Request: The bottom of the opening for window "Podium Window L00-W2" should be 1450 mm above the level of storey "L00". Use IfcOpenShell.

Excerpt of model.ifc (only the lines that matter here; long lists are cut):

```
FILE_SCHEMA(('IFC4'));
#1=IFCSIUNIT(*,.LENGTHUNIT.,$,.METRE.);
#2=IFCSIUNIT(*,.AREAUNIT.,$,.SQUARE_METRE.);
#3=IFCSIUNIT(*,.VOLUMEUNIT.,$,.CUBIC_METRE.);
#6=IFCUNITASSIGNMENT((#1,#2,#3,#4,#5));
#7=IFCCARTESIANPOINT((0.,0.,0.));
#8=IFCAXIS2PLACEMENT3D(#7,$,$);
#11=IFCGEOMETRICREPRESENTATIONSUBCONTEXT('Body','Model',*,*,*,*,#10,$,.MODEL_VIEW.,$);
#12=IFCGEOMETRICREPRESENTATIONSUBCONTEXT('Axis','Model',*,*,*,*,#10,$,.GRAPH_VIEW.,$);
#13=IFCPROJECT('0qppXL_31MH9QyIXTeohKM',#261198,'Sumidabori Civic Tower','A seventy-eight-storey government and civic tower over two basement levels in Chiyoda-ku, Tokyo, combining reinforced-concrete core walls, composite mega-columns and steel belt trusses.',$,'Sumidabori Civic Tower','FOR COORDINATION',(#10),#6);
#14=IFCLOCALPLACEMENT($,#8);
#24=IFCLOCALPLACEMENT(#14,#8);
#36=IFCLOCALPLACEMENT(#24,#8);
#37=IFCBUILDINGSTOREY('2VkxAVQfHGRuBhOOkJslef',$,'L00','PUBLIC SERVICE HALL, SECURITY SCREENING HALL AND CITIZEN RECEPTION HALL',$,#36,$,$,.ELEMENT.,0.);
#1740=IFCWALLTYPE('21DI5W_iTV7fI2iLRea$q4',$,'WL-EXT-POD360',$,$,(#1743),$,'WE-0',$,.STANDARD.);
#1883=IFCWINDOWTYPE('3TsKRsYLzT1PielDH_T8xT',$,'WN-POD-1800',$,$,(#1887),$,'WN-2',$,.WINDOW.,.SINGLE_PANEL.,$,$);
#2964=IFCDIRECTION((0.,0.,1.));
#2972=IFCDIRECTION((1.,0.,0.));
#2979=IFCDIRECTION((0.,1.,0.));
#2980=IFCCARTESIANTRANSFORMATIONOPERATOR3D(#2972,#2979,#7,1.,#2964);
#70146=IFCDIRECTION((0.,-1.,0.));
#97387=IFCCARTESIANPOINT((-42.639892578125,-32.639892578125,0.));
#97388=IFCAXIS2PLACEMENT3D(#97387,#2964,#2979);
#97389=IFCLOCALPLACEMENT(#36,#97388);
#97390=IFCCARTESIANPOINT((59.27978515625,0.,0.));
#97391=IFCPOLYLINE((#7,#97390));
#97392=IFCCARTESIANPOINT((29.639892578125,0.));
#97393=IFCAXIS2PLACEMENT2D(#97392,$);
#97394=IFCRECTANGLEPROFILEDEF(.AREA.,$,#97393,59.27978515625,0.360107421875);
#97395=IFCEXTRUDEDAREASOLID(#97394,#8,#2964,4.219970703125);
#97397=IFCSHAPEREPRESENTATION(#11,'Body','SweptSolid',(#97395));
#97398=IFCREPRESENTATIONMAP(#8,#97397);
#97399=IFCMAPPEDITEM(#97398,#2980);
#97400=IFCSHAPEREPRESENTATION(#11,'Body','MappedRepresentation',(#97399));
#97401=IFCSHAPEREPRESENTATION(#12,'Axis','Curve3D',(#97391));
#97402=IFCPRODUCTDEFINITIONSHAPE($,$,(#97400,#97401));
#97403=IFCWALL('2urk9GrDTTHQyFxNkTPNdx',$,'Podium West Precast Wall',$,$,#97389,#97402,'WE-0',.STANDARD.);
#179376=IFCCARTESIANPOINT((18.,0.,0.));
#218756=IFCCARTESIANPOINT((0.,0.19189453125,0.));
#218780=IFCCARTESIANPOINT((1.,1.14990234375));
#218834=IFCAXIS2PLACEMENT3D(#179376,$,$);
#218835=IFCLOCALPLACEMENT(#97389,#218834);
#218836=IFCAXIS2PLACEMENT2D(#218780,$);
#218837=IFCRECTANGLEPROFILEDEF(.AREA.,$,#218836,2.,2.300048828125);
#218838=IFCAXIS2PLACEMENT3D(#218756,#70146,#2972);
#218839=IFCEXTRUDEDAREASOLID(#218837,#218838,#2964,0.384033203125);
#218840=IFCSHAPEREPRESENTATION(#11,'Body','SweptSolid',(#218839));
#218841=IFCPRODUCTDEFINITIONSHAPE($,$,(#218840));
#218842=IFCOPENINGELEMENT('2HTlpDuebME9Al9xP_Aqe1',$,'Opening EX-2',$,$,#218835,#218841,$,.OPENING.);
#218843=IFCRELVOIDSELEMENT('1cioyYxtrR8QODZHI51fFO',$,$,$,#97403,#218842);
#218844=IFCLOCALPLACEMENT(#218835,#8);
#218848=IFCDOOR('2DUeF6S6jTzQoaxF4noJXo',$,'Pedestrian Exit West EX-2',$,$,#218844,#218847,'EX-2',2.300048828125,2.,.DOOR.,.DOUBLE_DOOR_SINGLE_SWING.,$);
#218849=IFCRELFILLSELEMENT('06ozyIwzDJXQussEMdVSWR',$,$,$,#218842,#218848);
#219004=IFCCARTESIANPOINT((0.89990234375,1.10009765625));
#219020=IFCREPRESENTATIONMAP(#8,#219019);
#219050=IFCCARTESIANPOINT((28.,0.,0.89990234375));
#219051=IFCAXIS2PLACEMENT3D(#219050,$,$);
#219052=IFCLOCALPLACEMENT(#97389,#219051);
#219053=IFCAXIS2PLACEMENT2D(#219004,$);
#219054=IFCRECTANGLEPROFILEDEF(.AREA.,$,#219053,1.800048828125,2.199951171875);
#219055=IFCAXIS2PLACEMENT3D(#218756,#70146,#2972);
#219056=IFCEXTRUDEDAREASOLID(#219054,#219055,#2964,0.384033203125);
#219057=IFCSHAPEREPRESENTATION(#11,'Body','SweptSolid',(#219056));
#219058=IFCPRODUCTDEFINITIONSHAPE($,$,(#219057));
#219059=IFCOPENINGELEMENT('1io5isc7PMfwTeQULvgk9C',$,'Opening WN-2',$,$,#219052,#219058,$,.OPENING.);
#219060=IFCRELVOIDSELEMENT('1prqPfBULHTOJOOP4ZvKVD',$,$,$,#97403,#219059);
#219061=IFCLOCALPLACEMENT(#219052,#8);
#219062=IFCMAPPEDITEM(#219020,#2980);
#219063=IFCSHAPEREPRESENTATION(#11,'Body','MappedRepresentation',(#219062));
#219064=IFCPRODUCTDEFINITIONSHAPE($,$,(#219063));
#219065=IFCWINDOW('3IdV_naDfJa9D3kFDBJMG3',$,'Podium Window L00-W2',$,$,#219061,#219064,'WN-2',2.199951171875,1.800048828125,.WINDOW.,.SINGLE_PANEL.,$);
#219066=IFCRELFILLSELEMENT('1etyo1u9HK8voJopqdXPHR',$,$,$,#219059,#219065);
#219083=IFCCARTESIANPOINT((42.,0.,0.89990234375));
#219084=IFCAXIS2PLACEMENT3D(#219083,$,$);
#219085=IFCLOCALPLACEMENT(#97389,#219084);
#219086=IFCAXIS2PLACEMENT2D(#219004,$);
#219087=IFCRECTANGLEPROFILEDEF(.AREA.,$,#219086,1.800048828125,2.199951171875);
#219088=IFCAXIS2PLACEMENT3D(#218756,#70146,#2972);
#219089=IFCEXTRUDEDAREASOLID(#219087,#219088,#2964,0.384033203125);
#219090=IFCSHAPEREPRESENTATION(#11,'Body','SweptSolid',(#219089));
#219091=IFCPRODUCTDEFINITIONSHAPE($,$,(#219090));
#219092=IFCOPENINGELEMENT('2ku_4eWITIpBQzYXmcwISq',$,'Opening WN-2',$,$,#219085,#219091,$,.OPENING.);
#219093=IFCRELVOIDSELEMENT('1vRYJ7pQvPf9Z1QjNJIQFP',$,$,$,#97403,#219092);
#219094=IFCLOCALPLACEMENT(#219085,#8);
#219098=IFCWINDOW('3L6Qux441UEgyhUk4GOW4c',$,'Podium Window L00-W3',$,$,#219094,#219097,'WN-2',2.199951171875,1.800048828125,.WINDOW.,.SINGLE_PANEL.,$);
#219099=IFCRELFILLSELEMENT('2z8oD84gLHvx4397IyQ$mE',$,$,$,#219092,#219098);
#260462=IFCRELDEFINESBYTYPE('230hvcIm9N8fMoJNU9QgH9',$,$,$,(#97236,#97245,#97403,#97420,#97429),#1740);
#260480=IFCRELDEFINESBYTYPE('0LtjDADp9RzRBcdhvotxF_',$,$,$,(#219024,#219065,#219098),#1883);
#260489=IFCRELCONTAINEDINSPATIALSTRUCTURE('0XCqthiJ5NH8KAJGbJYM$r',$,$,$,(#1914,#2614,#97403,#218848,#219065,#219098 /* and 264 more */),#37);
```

```python
import numpy as np
import ifcopenshell
import ifcopenshell.api.geometry
import ifcopenshell.geom
import ifcopenshell.util.element
import ifcopenshell.util.placement
import ifcopenshell.util.shape
import ifcopenshell.util.unit

model = ifcopenshell.open("model.ifc")
unit_scale = ifcopenshell.util.unit.calculate_unit_scale(model)

window = model.by_guid("3IdV_naDfJa9D3kFDBJMG3")
opening = window.FillsVoids[0].RelatingOpeningElement
storey = ifcopenshell.util.element.get_container(window, ifc_class="IfcBuildingStorey")
level = ifcopenshell.util.placement.get_local_placement(storey.ObjectPlacement)[2, 3]

# The opening's origin need not be at the sill, so measure its lowest point.
shape = ifcopenshell.geom.create_shape(ifcopenshell.geom.settings(), opening)
bottom = ifcopenshell.util.shape.get_shape_bottom_elevation(shape, shape.geometry) / unit_scale
dz = level + 1.45 / unit_scale - bottom

shift = np.array([0.0, 0.0, dz])
# The window is placed relative to its opening, so it follows when the opening moves.
matrix = ifcopenshell.util.placement.get_local_placement(opening.ObjectPlacement)
matrix[:3, 3] += shift
ifcopenshell.api.geometry.edit_object_placement(
    model, product=opening, matrix=matrix, is_si=False, should_transform_children=True
)

print(f"moved by {dz * unit_scale:+.3f} m")

model.write("model_rev.ifc")
```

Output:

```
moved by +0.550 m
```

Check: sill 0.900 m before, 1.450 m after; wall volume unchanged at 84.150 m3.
